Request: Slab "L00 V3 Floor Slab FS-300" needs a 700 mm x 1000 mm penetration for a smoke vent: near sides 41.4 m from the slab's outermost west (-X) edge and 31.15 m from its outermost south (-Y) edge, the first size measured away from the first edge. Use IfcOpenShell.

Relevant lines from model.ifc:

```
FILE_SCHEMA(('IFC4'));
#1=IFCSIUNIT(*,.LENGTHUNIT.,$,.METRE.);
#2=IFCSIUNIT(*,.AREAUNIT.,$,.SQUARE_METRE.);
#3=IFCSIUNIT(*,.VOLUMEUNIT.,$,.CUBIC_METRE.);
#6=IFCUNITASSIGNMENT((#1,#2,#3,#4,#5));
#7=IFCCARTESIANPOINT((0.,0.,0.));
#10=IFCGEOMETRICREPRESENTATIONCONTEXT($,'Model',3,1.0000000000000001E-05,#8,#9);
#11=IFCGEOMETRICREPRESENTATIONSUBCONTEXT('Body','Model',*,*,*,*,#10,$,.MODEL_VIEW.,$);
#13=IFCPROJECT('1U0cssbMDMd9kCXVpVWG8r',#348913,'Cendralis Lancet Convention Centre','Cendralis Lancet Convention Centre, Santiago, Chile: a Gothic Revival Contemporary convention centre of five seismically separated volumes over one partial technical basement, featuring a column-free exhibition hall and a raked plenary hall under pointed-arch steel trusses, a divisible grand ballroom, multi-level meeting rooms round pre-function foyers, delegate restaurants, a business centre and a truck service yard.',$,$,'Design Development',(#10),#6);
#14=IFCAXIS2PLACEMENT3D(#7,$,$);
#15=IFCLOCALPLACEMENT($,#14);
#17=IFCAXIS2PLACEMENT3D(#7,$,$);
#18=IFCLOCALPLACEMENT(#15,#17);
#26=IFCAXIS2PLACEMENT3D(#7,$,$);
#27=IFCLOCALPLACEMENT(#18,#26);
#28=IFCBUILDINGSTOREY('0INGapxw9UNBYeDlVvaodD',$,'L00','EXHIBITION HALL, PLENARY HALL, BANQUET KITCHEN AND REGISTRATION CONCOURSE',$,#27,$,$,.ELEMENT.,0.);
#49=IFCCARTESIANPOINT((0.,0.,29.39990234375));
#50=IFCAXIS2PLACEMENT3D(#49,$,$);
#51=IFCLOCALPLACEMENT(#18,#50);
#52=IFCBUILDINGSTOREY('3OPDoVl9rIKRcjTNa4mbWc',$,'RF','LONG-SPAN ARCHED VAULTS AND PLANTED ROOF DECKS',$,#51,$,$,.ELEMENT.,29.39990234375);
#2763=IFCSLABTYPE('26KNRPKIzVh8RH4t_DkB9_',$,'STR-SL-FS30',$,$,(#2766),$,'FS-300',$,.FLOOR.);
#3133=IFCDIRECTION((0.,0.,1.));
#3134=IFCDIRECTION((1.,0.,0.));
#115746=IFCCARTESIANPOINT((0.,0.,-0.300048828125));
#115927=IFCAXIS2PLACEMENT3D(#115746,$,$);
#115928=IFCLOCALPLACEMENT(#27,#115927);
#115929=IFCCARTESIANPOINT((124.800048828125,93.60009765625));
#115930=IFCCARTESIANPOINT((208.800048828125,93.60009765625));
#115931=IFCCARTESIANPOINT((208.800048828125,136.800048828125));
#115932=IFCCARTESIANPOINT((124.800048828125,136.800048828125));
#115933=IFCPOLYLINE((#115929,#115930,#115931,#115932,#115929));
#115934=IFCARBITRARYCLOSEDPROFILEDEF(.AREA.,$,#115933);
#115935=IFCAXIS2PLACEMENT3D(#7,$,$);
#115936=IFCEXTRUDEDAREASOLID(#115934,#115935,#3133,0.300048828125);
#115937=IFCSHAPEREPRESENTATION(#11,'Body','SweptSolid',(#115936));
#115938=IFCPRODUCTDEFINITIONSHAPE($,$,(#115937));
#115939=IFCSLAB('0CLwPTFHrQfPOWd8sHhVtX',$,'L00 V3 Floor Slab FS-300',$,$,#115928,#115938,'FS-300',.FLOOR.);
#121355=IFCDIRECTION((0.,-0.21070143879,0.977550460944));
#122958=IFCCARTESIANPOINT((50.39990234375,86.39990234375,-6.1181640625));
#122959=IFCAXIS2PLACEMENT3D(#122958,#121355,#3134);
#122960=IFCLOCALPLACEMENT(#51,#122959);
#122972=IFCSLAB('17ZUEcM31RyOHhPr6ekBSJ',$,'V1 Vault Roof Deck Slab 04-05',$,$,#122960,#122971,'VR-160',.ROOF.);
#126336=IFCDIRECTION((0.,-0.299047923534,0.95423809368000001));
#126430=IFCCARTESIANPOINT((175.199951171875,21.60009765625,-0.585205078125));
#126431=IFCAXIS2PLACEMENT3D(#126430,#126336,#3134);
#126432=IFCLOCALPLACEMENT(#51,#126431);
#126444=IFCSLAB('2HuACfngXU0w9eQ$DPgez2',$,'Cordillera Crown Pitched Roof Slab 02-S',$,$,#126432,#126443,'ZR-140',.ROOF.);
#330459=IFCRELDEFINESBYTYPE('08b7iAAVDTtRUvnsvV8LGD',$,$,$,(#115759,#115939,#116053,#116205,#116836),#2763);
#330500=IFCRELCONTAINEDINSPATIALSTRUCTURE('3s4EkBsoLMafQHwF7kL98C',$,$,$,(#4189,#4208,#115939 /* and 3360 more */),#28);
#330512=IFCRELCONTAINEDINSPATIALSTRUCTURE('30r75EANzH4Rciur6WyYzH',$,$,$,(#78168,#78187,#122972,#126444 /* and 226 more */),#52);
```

```python
import numpy as np
import ifcopenshell
import ifcopenshell.api.feature
import ifcopenshell.api.geometry
import ifcopenshell.api.root
import ifcopenshell.geom
import ifcopenshell.util.placement
import ifcopenshell.util.representation
import ifcopenshell.util.shape
import ifcopenshell.util.unit

model = ifcopenshell.open("model.ifc")
unit_scale = ifcopenshell.util.unit.calculate_unit_scale(model)
settings = ifcopenshell.geom.settings()


def volume(element):
    """Net volume in cubic metres, openings subtracted."""
    shape = ifcopenshell.geom.create_shape(settings, element)
    return ifcopenshell.util.shape.get_volume(shape.geometry)


slab = model.by_guid("0CLwPTFHrQfPOWd8sHhVtX")
before = volume(slab)

# Extent in the slab's own axes, in metres. The edges named are its -X and -Y sides.
slab_shape = ifcopenshell.geom.create_shape(settings, slab)
vertices = ifcopenshell.util.shape.get_vertices(slab_shape.geometry)
x_min, y_min, bottom = vertices.min(axis=0)
top = vertices[:, 2].max()

opening = ifcopenshell.api.root.create_entity(model, ifc_class="IfcOpeningElement", name="Smoke vent opening", predefined_type="OPENING")
context = ifcopenshell.util.representation.get_context(model, "Model", "Body", "MODEL_VIEW")
width, depth = 0.7, 1
outline = [(0.0, 0.0), (width, 0.0), (width, depth), (0.0, depth), (0.0, 0.0)]
# Overshoot both faces by 50 mm so the cut is clean.
shape = ifcopenshell.api.geometry.add_slab_representation(
    model, context=context, depth=top - bottom + 0.1, polyline=outline
)
ifcopenshell.api.geometry.assign_representation(model, product=opening, representation=shape)

matrix = ifcopenshell.util.placement.get_local_placement(slab.ObjectPlacement)
matrix[:, 3] = matrix @ np.append(np.array([x_min + 41.4, y_min + 31.15, bottom - 0.05]) / unit_scale, 1.0)
ifcopenshell.api.geometry.edit_object_placement(model, product=opening, matrix=matrix, is_si=False)
ifcopenshell.api.feature.add_feature(model, feature=opening, element=slab)

after = volume(slab)

print(f"slab volume {before:.3f} -> {after:.3f} m3")

model.write("model_v2.ifc")
```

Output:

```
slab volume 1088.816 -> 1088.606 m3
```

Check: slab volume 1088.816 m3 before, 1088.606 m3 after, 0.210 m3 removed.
